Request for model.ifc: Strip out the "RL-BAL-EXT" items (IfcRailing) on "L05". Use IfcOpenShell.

First a look at what the model holds.

```python
import ifcopenshell
import ifcopenshell.util.element

model = ifcopenshell.open("model.ifc")
print(model.schema)
storey = next(s for s in model.by_type("IfcBuildingStorey") if s.Name == "L05")
railings = [e for e in ifcopenshell.util.element.get_decomposition(storey) if e.is_a("IfcRailing")]
seen = {}
for e in railings:
    element_type = ifcopenshell.util.element.get_type(e)
    name = element_type.Name if element_type not in (None, e) else None
    seen[name] = seen.get(name, 0) + 1
for name, count in sorted(seen.items(), key=str):
    print(count, "x", name)
```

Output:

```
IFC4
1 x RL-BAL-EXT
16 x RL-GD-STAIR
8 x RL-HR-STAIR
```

```python
import ifcopenshell
import ifcopenshell.api.root
import ifcopenshell.util.element

model = ifcopenshell.open("model.ifc")

storey = next(s for s in model.by_type("IfcBuildingStorey") if s.Name == "L05")
railings = [e for e in ifcopenshell.util.element.get_decomposition(storey) if e.is_a("IfcRailing")]
targets = [e for e in railings if (t := ifcopenshell.util.element.get_type(e)) not in (None, e) and t.Name == "RL-BAL-EXT"]

for e in targets:
    ifcopenshell.api.root.remove_product(model, product=e)
print(len(targets), "removed")

model.write("model_edited.ifc")
```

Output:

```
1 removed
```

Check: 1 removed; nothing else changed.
